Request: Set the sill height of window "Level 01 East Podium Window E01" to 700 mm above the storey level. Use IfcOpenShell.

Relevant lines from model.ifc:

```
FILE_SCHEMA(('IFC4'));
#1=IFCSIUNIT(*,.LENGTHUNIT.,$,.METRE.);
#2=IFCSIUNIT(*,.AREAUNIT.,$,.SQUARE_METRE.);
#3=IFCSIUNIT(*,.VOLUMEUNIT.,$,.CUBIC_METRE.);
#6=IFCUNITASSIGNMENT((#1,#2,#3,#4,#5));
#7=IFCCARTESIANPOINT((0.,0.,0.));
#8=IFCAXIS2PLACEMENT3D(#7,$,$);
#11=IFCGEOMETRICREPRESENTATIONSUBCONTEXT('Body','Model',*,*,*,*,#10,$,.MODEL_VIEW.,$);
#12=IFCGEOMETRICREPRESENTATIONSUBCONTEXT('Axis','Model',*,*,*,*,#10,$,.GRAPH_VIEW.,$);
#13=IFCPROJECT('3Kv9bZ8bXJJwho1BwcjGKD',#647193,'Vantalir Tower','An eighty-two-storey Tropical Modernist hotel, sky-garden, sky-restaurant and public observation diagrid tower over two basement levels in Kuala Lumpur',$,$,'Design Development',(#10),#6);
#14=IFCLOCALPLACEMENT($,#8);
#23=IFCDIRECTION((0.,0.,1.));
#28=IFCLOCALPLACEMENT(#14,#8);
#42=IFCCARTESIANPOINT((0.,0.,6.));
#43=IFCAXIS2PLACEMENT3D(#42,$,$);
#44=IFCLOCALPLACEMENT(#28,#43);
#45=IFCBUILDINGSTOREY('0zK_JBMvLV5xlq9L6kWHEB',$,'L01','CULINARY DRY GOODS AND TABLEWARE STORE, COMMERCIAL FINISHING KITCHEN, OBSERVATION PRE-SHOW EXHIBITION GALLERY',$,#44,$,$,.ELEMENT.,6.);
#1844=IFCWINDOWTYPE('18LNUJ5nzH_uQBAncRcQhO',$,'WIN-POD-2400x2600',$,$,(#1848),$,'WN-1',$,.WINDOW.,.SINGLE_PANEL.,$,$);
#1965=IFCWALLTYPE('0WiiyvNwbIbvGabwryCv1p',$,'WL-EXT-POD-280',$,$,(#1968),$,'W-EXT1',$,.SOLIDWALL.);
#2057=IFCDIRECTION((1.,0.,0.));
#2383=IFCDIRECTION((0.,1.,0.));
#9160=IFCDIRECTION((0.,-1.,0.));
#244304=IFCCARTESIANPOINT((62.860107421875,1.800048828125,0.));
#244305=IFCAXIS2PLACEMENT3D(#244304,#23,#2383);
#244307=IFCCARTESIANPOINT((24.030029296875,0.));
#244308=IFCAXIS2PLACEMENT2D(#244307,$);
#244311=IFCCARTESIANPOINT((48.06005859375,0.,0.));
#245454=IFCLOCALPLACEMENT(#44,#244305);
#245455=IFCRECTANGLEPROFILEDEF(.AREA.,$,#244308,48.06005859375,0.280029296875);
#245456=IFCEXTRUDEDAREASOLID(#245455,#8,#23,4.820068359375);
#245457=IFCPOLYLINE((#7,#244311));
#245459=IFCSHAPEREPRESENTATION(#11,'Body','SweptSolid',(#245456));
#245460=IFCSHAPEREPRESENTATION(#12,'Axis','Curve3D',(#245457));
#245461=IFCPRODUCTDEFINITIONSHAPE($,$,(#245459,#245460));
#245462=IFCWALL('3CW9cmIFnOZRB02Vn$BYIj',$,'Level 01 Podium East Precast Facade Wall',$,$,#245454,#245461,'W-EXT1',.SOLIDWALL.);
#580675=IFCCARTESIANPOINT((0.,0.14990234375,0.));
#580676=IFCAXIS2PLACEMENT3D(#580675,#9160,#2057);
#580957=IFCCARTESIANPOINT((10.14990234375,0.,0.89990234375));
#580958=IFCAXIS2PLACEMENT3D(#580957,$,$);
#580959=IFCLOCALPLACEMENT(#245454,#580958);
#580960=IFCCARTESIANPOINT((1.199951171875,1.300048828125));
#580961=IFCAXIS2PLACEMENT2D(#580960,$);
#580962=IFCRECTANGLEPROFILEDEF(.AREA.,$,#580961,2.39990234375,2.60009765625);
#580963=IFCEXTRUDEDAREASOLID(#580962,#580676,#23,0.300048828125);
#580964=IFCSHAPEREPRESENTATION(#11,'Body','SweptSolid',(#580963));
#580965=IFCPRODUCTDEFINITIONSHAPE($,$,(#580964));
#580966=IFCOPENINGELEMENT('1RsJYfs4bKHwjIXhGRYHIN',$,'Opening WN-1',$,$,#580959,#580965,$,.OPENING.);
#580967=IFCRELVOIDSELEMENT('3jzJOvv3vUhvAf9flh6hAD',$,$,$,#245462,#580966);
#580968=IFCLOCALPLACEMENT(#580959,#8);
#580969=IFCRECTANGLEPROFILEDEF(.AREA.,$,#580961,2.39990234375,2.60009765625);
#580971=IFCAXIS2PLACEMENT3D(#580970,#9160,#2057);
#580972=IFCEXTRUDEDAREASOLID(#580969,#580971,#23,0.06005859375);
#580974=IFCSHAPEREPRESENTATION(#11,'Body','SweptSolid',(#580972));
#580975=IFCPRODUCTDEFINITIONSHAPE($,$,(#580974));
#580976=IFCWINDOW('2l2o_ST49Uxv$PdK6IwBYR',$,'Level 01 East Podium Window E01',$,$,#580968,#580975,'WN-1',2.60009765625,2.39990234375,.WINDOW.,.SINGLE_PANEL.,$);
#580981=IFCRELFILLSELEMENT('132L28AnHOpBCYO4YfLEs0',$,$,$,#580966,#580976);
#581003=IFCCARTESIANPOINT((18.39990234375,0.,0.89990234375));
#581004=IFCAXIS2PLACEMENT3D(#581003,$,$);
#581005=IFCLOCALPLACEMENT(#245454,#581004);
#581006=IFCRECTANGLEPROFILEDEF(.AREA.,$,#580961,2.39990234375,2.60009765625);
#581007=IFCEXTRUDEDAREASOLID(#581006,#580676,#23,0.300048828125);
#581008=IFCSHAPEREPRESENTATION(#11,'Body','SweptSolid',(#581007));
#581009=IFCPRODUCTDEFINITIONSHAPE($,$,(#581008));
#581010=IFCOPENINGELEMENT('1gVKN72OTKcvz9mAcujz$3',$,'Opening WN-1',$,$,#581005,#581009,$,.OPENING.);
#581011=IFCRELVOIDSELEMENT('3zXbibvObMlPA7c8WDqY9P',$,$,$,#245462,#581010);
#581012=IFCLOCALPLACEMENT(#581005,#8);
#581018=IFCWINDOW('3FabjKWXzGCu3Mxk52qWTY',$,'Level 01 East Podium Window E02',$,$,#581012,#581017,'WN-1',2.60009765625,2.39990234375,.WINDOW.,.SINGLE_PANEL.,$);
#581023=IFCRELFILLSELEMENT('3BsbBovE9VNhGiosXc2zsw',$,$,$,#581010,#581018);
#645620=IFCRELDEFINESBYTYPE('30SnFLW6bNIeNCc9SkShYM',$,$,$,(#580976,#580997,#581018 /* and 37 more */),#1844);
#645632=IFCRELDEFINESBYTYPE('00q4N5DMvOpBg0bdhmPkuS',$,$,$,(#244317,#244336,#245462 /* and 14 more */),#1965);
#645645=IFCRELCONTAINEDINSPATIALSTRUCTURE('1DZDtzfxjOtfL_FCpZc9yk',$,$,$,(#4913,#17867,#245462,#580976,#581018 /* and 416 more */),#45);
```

```python
import numpy as np
import ifcopenshell
import ifcopenshell.api.geometry
import ifcopenshell.geom
import ifcopenshell.util.element
import ifcopenshell.util.placement
import ifcopenshell.util.shape
import ifcopenshell.util.unit

model = ifcopenshell.open("model.ifc")
unit_scale = ifcopenshell.util.unit.calculate_unit_scale(model)

window = model.by_id(580976)
opening = window.FillsVoids[0].RelatingOpeningElement
storey = ifcopenshell.util.element.get_container(window, ifc_class="IfcBuildingStorey")
level = ifcopenshell.util.placement.get_local_placement(storey.ObjectPlacement)[2, 3]

# The opening's origin need not be at the sill, so measure its lowest point.
shape = ifcopenshell.geom.create_shape(ifcopenshell.geom.settings(), opening)
bottom = ifcopenshell.util.shape.get_shape_bottom_elevation(shape, shape.geometry) / unit_scale
dz = level + 0.7 - bottom

shift = np.array([0.0, 0.0, dz])
# The window is placed relative to its opening, so it follows when the opening moves.
matrix = ifcopenshell.util.placement.get_local_placement(opening.ObjectPlacement)
matrix[:3, 3] += shift
ifcopenshell.api.geometry.edit_object_placement(
    model, product=opening, matrix=matrix, is_si=False, should_transform_children=True
)

print(f"moved by {dz * unit_scale:+.3f} m")

model.write("model-out.ifc")
```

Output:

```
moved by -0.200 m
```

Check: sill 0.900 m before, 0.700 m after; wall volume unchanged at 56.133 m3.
